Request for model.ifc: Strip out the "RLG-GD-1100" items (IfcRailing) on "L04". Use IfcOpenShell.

First a look at what the model holds.

```python
import ifcopenshell
import ifcopenshell.util.element

model = ifcopenshell.open("model.ifc")
print(model.schema)
storey = next(s for s in model.by_type("IfcBuildingStorey") if s.Name == "L04")
railings = [e for e in ifcopenshell.util.element.get_decomposition(storey) if e.is_a("IfcRailing")]
seen = {}
for e in railings:
    element_type = ifcopenshell.util.element.get_type(e)
    name = element_type.Name if element_type not in (None, e) else None
    seen[name] = seen.get(name, 0) + 1
for name, count in sorted(seen.items(), key=str):
    print(count, "x", name)
```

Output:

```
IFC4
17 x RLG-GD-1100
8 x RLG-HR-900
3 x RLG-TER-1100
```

```python
import ifcopenshell
import ifcopenshell.api.root
import ifcopenshell.util.element

model = ifcopenshell.open("model.ifc")

storey = next(s for s in model.by_type("IfcBuildingStorey") if s.Name == "L04")
railings = [e for e in ifcopenshell.util.element.get_decomposition(storey) if e.is_a("IfcRailing")]
targets = [e for e in railings if (t := ifcopenshell.util.element.get_type(e)) not in (None, e) and t.Name == "RLG-GD-1100"]

for e in targets:
    ifcopenshell.api.root.remove_product(model, product=e)
print(len(targets), "removed")

model.write("model-out.ifc")
```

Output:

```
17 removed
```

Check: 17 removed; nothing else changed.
